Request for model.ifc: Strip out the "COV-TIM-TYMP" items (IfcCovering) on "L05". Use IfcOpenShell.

First a look at what the model holds.

```python
import ifcopenshell
import ifcopenshell.util.element

model = ifcopenshell.open("model.ifc")
print(model.schema)
storey = next(s for s in model.by_type("IfcBuildingStorey") if s.Name == "L05")
coverings = [e for e in ifcopenshell.util.element.get_decomposition(storey) if e.is_a("IfcCovering")]
seen = {}
for e in coverings:
    element_type = ifcopenshell.util.element.get_type(e)
    name = element_type.Name if element_type not in (None, e) else None
    seen[name] = seen.get(name, 0) + 1
for name, count in sorted(seen.items(), key=str):
    print(count, "x", name)
```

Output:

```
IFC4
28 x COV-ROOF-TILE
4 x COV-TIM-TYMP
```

```python
import ifcopenshell
import ifcopenshell.api.root
import ifcopenshell.util.element

model = ifcopenshell.open("model.ifc")

storey = next(s for s in model.by_type("IfcBuildingStorey") if s.Name == "L05")
coverings = [e for e in ifcopenshell.util.element.get_decomposition(storey) if e.is_a("IfcCovering")]
targets = [e for e in coverings if (t := ifcopenshell.util.element.get_type(e)) not in (None, e) and t.Name == "COV-TIM-TYMP"]

for e in targets:
    ifcopenshell.api.root.remove_product(model, product=e)
print(len(targets), "removed")

model.write("model_v2.ifc")
```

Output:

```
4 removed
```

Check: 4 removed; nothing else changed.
